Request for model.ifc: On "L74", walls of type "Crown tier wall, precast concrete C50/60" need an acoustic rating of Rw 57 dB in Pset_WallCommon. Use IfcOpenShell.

First a look at what the model holds.

```python
import ifcopenshell
import ifcopenshell.util.element

model = ifcopenshell.open("model.ifc")
print(model.schema)
storey = next(s for s in model.by_type("IfcBuildingStorey") if s.Name == "L74")
walls = [e for e in ifcopenshell.util.element.get_decomposition(storey) if e.is_a("IfcWall")]
seen = {}
for e in walls:
    element_type = ifcopenshell.util.element.get_type(e)
    key = (element_type.Name if element_type != e and element_type else None, ifcopenshell.util.element.get_pset(e, "Pset_WallCommon", "AcousticRating"))
    seen[key] = seen.get(key, 0) + 1
for (name, value), count in sorted(seen.items(), key=str):
    print(count, "x", name, "|", value)
```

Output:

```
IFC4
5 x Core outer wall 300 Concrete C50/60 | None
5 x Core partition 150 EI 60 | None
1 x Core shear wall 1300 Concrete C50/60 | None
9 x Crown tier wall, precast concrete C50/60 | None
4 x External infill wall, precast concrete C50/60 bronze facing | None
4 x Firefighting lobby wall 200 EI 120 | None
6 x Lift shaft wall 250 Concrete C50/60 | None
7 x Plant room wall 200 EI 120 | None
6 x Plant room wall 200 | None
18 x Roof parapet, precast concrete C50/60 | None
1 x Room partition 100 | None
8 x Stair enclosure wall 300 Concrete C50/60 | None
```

```python
import ifcopenshell
import ifcopenshell.api.pset
import ifcopenshell.util.element

model = ifcopenshell.open("model.ifc")

storey = next(s for s in model.by_type("IfcBuildingStorey") if s.Name == "L74")
walls = [e for e in ifcopenshell.util.element.get_decomposition(storey) if e.is_a("IfcWall")]

count = 0
for e in walls:
    element_type = ifcopenshell.util.element.get_type(e)
    if element_type in (None, e) or element_type.Name != "Crown tier wall, precast concrete C50/60":
        continue
    found = ifcopenshell.util.element.get_pset(e, "Pset_WallCommon", should_inherit=False)
    if found:
        pset = model.by_id(found["id"])
        if len(ifcopenshell.util.element.get_elements_by_pset(pset)) > 1:
            pset = ifcopenshell.api.pset.unshare_pset(model, products=[e], pset=pset)[0]
    else:
        pset = ifcopenshell.api.pset.add_pset(model, product=e, name="Pset_WallCommon")
    ifcopenshell.api.pset.edit_pset(model, pset=pset, properties={"AcousticRating": "Rw 57 dB"})
    count += 1

print(count, "walls updated")

model.write("model_v2.ifc")
```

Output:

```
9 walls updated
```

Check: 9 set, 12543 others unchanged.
